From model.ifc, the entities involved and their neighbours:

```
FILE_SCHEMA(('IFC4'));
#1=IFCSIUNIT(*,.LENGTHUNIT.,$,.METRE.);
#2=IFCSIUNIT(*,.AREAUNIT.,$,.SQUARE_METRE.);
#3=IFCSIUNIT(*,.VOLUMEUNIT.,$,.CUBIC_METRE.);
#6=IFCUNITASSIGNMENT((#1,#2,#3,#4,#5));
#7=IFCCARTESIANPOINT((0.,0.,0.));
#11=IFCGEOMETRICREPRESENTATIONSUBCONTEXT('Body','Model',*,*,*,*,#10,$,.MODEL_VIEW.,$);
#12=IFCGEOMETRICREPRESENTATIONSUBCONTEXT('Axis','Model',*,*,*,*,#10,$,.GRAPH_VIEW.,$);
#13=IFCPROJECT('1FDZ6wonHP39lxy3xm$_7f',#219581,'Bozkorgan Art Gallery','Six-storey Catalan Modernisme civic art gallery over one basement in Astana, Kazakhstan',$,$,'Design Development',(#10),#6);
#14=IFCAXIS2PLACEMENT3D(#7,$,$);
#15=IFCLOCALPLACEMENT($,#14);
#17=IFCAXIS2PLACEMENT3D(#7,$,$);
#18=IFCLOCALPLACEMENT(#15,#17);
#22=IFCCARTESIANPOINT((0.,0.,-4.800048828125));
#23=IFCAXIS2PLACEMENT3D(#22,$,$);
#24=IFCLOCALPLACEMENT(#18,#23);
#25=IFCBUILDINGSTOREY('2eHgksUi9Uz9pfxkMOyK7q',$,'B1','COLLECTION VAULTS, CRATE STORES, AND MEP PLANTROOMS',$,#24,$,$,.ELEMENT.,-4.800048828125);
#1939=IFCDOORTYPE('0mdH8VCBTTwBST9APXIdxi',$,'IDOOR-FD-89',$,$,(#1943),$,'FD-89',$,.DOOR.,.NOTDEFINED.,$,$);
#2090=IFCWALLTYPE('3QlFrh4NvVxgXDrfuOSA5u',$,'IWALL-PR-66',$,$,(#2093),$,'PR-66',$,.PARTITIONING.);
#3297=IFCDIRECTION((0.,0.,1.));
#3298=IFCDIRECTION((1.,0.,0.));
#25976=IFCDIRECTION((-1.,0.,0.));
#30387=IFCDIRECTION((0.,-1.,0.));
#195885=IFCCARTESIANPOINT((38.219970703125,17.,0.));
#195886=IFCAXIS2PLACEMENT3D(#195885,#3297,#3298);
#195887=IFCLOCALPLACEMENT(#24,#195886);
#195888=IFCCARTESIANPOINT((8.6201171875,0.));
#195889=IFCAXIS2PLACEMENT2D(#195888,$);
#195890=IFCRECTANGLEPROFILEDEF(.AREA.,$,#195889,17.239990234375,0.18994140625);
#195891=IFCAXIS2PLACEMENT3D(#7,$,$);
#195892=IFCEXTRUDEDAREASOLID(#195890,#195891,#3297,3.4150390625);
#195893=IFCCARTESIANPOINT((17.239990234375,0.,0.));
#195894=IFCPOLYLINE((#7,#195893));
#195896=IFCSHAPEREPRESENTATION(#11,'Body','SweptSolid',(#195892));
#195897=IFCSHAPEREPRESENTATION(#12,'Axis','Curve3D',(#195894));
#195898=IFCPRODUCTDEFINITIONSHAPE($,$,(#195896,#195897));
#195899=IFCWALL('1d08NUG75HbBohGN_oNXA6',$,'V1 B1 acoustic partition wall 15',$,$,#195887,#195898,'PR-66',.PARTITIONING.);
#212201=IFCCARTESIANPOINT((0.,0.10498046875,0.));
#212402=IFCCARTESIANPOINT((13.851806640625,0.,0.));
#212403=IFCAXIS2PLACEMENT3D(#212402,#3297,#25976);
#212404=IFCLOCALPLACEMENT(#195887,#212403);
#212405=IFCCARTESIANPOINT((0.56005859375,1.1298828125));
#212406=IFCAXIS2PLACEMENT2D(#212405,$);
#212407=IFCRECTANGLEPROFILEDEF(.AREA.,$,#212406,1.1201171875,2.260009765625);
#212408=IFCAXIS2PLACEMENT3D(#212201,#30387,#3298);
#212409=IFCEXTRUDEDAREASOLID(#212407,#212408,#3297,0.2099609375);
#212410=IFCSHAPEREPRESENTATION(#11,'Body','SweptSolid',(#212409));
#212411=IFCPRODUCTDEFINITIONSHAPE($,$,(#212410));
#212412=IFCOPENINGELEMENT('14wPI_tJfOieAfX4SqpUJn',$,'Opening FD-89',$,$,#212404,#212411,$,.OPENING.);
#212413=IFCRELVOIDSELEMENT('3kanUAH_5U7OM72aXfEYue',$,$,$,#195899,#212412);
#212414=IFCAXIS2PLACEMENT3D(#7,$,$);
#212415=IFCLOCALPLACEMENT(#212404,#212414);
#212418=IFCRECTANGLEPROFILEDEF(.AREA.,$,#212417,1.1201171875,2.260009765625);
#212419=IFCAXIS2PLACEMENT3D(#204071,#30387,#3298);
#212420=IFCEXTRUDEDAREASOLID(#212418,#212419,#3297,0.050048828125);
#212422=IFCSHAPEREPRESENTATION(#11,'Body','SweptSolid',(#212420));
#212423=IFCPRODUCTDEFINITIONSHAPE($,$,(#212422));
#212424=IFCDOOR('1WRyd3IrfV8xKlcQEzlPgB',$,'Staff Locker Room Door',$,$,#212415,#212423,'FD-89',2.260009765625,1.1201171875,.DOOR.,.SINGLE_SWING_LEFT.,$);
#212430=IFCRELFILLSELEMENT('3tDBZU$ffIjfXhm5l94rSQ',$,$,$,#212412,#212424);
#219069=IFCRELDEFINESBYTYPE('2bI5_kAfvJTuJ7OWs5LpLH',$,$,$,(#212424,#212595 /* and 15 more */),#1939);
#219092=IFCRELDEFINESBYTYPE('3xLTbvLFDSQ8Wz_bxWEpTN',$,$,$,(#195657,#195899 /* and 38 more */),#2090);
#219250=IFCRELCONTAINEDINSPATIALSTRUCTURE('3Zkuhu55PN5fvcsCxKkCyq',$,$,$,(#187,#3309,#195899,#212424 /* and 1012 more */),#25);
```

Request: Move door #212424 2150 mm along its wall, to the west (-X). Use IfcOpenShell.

```python
import ifcopenshell
import ifcopenshell.api.geometry
import ifcopenshell.util.placement
import ifcopenshell.util.unit

model = ifcopenshell.open("model.ifc")
unit_scale = ifcopenshell.util.unit.calculate_unit_scale(model)

door = model.by_guid("1WRyd3IrfV8xKlcQEzlPgB")
opening = door.FillsVoids[0].RelatingOpeningElement
wall = opening.VoidsElements[0].RelatingBuildingElement

wall_matrix = ifcopenshell.util.placement.get_local_placement(wall.ObjectPlacement)
shift = wall_matrix[:3, 0] * -2.15 / unit_scale
before = ifcopenshell.util.placement.get_local_placement(door.ObjectPlacement)[:3, 3].copy()

# The door is placed relative to its opening, so it follows when the opening moves.
matrix = ifcopenshell.util.placement.get_local_placement(opening.ObjectPlacement)
matrix[:3, 3] += shift
ifcopenshell.api.geometry.edit_object_placement(
    model, product=opening, matrix=matrix, is_si=False, should_transform_children=True
)

after = ifcopenshell.util.placement.get_local_placement(door.ObjectPlacement)[:3, 3]
print("door moved by", (after - before).round(3) + 0.0)

model.write("model_edited.ifc")
```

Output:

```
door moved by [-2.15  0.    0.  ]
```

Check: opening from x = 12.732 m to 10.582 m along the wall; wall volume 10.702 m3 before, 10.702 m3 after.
